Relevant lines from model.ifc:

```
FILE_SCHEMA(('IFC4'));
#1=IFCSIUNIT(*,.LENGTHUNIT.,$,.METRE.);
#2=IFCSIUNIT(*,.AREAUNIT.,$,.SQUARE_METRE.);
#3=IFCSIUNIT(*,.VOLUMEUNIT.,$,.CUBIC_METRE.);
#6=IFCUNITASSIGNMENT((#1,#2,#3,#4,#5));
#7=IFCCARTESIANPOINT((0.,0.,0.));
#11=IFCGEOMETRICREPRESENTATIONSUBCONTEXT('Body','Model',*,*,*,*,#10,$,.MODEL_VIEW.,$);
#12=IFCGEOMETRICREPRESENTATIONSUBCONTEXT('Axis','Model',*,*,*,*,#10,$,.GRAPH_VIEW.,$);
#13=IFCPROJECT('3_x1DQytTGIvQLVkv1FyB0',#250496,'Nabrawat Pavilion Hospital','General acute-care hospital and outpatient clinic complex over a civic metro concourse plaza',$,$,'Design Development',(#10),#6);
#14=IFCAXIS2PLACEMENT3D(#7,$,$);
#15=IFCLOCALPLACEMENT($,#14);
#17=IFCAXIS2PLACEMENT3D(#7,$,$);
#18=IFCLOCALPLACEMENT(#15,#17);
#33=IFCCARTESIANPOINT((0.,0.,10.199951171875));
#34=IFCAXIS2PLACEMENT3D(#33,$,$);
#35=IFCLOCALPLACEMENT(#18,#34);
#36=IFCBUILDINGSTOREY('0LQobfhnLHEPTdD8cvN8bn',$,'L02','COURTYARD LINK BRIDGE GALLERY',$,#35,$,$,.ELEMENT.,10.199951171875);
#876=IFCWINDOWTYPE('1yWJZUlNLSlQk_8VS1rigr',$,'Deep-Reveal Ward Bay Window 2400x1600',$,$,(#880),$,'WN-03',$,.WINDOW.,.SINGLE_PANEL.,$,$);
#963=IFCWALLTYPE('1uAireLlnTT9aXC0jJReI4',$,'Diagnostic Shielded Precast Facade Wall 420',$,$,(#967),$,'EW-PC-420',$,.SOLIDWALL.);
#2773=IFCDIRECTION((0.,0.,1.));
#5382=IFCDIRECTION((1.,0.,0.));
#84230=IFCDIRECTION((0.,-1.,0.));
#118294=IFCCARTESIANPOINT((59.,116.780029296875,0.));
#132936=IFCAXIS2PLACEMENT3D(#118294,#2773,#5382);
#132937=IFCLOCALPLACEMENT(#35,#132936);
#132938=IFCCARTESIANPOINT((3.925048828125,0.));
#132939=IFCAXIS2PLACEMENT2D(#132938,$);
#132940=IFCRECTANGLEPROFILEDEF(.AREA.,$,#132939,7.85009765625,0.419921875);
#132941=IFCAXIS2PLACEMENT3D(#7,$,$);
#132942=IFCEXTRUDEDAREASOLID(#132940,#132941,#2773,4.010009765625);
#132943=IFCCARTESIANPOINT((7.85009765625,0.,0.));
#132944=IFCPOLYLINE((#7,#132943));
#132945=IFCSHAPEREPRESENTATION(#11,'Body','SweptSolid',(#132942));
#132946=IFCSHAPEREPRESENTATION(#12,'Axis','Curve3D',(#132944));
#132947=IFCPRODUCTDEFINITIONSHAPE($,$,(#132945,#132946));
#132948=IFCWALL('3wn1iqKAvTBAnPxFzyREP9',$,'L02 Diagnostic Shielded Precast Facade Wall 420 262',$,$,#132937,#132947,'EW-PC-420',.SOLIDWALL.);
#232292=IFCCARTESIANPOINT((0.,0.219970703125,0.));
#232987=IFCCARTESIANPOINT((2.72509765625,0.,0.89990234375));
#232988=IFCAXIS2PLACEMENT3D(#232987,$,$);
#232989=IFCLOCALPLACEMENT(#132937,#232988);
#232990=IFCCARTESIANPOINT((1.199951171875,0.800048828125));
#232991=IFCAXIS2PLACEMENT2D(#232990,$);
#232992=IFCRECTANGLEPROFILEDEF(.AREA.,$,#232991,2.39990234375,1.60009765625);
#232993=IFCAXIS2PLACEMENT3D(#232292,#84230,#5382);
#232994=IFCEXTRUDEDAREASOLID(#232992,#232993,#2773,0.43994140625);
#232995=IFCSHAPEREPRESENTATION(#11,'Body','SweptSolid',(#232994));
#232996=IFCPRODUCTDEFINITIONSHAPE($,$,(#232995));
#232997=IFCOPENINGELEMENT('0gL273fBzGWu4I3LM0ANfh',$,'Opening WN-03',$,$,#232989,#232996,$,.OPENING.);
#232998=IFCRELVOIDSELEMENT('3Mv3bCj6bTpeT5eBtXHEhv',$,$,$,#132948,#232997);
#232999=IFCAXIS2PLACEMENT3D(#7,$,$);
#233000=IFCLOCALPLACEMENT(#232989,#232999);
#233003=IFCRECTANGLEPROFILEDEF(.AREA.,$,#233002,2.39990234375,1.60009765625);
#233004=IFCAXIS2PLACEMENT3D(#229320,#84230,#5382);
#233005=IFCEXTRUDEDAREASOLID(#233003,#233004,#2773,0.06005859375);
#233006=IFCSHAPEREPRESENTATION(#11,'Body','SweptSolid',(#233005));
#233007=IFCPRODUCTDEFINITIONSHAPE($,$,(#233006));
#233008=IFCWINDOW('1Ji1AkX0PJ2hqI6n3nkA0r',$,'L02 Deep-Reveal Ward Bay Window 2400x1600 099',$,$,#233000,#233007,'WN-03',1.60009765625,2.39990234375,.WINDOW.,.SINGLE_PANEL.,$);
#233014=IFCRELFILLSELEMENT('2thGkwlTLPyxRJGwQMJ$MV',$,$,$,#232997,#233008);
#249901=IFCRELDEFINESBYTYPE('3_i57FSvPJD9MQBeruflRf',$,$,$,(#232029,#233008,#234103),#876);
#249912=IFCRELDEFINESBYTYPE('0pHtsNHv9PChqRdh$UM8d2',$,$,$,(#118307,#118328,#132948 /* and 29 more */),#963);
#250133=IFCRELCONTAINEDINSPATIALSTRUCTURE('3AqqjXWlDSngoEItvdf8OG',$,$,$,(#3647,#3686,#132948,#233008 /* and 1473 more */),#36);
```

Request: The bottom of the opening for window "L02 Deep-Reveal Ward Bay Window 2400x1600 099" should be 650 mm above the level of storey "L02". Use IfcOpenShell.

```python
import numpy as np
import ifcopenshell
import ifcopenshell.api.geometry
import ifcopenshell.geom
import ifcopenshell.util.element
import ifcopenshell.util.placement
import ifcopenshell.util.shape
import ifcopenshell.util.unit

model = ifcopenshell.open("model.ifc")
unit_scale = ifcopenshell.util.unit.calculate_unit_scale(model)

window = model.by_id(233008)
opening = window.FillsVoids[0].RelatingOpeningElement
storey = ifcopenshell.util.element.get_container(window, ifc_class="IfcBuildingStorey")
level = ifcopenshell.util.placement.get_local_placement(storey.ObjectPlacement)[2, 3]

# The opening's origin need not be at the sill, so measure its lowest point.
shape = ifcopenshell.geom.create_shape(ifcopenshell.geom.settings(), opening)
bottom = ifcopenshell.util.shape.get_shape_bottom_elevation(shape, shape.geometry) / unit_scale
dz = level + 0.65 / unit_scale - bottom

shift = np.array([0.0, 0.0, dz])
# The window is placed relative to its opening, so it follows when the opening moves.
matrix = ifcopenshell.util.placement.get_local_placement(opening.ObjectPlacement)
matrix[:3, 3] += shift
ifcopenshell.api.geometry.edit_object_placement(
    model, product=opening, matrix=matrix, is_si=False, should_transform_children=True
)

print(f"moved by {dz * unit_scale:+.3f} m")

model.write("model_v2.ifc")
```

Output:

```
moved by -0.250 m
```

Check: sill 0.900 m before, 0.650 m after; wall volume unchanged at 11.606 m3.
